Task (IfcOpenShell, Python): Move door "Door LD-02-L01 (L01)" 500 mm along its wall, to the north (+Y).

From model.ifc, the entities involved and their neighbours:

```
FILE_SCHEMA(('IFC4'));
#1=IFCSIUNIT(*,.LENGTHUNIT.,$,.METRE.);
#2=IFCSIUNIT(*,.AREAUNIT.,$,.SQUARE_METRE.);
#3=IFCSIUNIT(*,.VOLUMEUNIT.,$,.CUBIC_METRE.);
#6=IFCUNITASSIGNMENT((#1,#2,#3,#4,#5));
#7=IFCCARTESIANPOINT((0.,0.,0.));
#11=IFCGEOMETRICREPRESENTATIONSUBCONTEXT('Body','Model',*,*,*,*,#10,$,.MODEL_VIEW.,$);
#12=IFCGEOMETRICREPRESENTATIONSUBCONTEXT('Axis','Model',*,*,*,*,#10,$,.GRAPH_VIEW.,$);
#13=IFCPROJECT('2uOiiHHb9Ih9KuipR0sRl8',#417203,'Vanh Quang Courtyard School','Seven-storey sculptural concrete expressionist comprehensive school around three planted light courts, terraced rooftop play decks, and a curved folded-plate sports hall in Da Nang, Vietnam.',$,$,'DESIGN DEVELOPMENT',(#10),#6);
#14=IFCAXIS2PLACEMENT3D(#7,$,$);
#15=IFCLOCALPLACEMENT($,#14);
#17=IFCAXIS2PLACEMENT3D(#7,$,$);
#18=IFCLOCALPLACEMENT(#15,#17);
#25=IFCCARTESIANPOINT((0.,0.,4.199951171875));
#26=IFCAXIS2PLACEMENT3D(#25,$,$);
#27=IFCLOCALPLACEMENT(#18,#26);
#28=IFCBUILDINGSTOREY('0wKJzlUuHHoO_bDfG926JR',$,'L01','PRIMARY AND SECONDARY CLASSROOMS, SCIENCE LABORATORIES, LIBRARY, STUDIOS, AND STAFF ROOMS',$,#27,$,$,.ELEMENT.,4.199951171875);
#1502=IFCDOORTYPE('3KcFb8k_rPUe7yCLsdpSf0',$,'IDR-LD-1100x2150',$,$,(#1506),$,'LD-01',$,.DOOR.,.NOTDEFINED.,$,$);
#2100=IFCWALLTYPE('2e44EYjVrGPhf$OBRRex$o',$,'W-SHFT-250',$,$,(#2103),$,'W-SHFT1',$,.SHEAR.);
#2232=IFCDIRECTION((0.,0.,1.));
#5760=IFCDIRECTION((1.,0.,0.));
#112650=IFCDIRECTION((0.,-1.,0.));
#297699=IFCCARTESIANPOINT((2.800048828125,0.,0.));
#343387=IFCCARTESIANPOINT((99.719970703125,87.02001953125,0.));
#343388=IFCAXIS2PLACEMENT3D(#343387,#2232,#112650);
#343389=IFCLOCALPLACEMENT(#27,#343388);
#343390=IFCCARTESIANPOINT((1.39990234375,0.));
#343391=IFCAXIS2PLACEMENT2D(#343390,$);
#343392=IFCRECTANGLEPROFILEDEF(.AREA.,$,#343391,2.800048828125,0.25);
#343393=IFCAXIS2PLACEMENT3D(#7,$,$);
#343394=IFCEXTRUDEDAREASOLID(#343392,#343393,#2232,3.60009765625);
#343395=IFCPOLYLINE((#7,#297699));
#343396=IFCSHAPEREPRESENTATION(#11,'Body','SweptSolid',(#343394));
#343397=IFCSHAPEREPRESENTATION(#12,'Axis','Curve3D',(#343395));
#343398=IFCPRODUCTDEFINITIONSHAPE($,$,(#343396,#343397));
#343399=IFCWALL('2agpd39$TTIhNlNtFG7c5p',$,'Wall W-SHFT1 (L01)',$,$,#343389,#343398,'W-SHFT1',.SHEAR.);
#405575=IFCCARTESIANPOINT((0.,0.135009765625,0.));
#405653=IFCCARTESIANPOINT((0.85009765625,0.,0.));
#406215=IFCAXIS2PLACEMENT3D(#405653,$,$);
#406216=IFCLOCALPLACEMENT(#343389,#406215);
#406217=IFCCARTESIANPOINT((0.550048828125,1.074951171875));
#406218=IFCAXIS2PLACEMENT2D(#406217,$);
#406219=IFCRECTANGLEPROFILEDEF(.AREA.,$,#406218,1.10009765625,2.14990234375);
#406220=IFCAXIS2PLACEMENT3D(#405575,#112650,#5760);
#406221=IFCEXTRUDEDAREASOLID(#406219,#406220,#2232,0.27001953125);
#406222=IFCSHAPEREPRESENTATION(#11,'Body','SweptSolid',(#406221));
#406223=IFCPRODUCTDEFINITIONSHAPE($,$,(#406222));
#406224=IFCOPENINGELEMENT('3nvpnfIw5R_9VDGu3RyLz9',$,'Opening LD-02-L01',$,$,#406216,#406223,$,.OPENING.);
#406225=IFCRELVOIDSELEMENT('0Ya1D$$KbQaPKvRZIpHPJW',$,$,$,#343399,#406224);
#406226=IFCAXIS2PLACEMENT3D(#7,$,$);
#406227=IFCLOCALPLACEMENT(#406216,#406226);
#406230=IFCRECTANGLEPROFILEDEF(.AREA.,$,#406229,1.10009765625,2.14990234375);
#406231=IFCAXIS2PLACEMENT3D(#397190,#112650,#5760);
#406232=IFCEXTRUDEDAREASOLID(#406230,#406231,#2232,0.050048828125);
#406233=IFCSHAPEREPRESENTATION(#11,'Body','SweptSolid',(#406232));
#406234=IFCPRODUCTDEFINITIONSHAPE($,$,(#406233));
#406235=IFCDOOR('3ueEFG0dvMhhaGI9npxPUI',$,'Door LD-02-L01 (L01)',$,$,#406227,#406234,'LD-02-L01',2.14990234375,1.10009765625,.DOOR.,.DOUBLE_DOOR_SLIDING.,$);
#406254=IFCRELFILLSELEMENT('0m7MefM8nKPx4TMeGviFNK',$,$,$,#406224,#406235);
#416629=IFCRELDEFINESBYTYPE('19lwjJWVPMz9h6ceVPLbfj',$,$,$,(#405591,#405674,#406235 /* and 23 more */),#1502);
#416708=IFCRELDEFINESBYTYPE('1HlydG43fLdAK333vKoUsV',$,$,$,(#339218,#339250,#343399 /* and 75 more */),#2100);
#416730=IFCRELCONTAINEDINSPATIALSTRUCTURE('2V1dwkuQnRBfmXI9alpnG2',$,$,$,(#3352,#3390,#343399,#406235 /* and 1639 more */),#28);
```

```python
import ifcopenshell
import ifcopenshell.api.geometry
import ifcopenshell.util.placement
import ifcopenshell.util.unit

model = ifcopenshell.open("model.ifc")
unit_scale = ifcopenshell.util.unit.calculate_unit_scale(model)

door = model.by_guid("3ueEFG0dvMhhaGI9npxPUI")
opening = door.FillsVoids[0].RelatingOpeningElement
wall = opening.VoidsElements[0].RelatingBuildingElement

wall_matrix = ifcopenshell.util.placement.get_local_placement(wall.ObjectPlacement)
shift = wall_matrix[:3, 0] * -0.5 / unit_scale
before = ifcopenshell.util.placement.get_local_placement(door.ObjectPlacement)[:3, 3].copy()

# The door is placed relative to its opening, so it follows when the opening moves.
matrix = ifcopenshell.util.placement.get_local_placement(opening.ObjectPlacement)
matrix[:3, 3] += shift
ifcopenshell.api.geometry.edit_object_placement(
    model, product=opening, matrix=matrix, is_si=False, should_transform_children=True
)

after = ifcopenshell.util.placement.get_local_placement(door.ObjectPlacement)[:3, 3]
print("door moved by", (after - before).round(3) + 0.0)

model.write("model_updated.ifc")
```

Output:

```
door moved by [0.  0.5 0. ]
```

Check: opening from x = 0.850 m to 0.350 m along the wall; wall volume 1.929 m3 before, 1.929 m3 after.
